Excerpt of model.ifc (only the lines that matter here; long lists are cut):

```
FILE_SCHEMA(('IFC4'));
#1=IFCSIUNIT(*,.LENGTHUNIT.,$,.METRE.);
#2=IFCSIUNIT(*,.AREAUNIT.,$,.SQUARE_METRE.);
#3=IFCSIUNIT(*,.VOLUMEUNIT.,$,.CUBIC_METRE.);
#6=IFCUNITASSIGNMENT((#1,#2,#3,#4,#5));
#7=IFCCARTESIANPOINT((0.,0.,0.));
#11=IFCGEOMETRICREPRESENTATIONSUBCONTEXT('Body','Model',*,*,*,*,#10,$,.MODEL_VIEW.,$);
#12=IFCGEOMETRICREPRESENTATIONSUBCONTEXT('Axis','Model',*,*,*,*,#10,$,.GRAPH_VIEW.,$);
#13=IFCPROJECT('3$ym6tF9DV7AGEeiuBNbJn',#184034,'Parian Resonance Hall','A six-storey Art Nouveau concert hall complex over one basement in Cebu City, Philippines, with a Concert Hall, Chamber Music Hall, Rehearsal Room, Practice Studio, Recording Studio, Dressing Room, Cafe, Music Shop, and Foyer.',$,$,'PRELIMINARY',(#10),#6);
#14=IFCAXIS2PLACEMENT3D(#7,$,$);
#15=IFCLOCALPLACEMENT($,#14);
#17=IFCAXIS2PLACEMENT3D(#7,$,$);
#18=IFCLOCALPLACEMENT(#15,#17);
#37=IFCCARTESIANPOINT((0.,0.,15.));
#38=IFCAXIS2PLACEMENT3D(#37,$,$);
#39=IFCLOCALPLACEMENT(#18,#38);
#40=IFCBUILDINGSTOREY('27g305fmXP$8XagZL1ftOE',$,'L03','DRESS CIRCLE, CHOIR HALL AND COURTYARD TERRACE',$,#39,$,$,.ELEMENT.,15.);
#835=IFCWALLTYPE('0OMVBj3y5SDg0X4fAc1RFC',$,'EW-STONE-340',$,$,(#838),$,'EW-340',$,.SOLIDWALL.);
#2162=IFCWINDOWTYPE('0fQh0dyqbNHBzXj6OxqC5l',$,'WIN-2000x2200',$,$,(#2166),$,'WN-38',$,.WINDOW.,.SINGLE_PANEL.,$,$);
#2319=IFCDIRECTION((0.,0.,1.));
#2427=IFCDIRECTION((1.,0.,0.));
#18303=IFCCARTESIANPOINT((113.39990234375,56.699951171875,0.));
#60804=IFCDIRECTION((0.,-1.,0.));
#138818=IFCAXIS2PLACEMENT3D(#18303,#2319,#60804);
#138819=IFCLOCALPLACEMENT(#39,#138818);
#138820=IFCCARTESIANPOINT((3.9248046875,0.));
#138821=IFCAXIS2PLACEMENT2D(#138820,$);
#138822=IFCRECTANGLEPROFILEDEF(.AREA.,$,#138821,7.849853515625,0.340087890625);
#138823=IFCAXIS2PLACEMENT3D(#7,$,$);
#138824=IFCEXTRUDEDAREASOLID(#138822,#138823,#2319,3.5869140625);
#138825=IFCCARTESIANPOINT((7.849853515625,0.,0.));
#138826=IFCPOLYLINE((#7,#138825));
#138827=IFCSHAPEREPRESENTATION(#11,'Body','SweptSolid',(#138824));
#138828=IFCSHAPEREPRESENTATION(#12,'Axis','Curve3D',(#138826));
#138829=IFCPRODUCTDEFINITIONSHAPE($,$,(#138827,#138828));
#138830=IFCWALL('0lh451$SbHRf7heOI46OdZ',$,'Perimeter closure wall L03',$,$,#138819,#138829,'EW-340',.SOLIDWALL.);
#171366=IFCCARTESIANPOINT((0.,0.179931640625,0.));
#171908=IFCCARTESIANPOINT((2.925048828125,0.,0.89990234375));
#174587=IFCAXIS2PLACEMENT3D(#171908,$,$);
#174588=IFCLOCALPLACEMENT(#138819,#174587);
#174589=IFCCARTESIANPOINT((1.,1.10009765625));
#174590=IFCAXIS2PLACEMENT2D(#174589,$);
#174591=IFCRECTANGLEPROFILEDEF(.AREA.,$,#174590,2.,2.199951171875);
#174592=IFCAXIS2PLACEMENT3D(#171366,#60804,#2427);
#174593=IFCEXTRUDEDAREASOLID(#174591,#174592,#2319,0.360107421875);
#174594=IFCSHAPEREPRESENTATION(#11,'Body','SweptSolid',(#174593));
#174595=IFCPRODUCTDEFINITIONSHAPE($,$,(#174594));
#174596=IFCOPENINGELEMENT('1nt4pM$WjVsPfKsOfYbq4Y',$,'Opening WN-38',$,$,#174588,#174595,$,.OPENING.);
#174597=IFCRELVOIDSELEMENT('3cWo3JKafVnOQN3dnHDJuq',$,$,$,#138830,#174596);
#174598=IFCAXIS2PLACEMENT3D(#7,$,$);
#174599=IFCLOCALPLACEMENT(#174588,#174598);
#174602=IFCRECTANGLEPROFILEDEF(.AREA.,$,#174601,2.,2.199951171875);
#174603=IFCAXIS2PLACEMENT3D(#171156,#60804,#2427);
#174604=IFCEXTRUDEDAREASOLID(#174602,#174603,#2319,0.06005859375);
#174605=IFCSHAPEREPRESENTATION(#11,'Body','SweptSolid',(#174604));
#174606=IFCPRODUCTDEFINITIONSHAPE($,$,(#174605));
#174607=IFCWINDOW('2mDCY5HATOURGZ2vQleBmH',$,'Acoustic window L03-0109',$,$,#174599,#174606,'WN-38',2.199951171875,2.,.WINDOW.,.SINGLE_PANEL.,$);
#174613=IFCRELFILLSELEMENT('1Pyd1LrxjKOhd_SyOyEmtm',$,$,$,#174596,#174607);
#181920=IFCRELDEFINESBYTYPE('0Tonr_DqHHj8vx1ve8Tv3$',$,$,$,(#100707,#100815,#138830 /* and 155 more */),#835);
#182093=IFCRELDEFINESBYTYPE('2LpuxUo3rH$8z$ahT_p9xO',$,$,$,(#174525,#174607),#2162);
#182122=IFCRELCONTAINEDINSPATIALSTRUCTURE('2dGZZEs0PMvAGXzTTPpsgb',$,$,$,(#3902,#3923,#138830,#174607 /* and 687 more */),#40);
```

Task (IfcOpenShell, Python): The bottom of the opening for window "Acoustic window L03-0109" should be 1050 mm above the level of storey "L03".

```python
import numpy as np
import ifcopenshell
import ifcopenshell.api.geometry
import ifcopenshell.geom
import ifcopenshell.util.element
import ifcopenshell.util.placement
import ifcopenshell.util.shape
import ifcopenshell.util.unit

model = ifcopenshell.open("model.ifc")
unit_scale = ifcopenshell.util.unit.calculate_unit_scale(model)

window = model.by_guid("2mDCY5HATOURGZ2vQleBmH")
opening = window.FillsVoids[0].RelatingOpeningElement
storey = ifcopenshell.util.element.get_container(window, ifc_class="IfcBuildingStorey")
level = ifcopenshell.util.placement.get_local_placement(storey.ObjectPlacement)[2, 3]

# The opening's origin need not be at the sill, so measure its lowest point.
shape = ifcopenshell.geom.create_shape(ifcopenshell.geom.settings(), opening)
bottom = ifcopenshell.util.shape.get_shape_bottom_elevation(shape, shape.geometry) / unit_scale
dz = level + 1.05 - bottom

shift = np.array([0.0, 0.0, dz])
# The window is placed relative to its opening, so it follows when the opening moves.
matrix = ifcopenshell.util.placement.get_local_placement(opening.ObjectPlacement)
matrix[:3, 3] += shift
ifcopenshell.api.geometry.edit_object_placement(
    model, product=opening, matrix=matrix, is_si=False, should_transform_children=True
)

print(f"moved by {dz * unit_scale:+.3f} m")

model.write("model_updated.ifc")
```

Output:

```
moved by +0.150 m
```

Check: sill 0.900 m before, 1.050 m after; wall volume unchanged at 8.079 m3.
